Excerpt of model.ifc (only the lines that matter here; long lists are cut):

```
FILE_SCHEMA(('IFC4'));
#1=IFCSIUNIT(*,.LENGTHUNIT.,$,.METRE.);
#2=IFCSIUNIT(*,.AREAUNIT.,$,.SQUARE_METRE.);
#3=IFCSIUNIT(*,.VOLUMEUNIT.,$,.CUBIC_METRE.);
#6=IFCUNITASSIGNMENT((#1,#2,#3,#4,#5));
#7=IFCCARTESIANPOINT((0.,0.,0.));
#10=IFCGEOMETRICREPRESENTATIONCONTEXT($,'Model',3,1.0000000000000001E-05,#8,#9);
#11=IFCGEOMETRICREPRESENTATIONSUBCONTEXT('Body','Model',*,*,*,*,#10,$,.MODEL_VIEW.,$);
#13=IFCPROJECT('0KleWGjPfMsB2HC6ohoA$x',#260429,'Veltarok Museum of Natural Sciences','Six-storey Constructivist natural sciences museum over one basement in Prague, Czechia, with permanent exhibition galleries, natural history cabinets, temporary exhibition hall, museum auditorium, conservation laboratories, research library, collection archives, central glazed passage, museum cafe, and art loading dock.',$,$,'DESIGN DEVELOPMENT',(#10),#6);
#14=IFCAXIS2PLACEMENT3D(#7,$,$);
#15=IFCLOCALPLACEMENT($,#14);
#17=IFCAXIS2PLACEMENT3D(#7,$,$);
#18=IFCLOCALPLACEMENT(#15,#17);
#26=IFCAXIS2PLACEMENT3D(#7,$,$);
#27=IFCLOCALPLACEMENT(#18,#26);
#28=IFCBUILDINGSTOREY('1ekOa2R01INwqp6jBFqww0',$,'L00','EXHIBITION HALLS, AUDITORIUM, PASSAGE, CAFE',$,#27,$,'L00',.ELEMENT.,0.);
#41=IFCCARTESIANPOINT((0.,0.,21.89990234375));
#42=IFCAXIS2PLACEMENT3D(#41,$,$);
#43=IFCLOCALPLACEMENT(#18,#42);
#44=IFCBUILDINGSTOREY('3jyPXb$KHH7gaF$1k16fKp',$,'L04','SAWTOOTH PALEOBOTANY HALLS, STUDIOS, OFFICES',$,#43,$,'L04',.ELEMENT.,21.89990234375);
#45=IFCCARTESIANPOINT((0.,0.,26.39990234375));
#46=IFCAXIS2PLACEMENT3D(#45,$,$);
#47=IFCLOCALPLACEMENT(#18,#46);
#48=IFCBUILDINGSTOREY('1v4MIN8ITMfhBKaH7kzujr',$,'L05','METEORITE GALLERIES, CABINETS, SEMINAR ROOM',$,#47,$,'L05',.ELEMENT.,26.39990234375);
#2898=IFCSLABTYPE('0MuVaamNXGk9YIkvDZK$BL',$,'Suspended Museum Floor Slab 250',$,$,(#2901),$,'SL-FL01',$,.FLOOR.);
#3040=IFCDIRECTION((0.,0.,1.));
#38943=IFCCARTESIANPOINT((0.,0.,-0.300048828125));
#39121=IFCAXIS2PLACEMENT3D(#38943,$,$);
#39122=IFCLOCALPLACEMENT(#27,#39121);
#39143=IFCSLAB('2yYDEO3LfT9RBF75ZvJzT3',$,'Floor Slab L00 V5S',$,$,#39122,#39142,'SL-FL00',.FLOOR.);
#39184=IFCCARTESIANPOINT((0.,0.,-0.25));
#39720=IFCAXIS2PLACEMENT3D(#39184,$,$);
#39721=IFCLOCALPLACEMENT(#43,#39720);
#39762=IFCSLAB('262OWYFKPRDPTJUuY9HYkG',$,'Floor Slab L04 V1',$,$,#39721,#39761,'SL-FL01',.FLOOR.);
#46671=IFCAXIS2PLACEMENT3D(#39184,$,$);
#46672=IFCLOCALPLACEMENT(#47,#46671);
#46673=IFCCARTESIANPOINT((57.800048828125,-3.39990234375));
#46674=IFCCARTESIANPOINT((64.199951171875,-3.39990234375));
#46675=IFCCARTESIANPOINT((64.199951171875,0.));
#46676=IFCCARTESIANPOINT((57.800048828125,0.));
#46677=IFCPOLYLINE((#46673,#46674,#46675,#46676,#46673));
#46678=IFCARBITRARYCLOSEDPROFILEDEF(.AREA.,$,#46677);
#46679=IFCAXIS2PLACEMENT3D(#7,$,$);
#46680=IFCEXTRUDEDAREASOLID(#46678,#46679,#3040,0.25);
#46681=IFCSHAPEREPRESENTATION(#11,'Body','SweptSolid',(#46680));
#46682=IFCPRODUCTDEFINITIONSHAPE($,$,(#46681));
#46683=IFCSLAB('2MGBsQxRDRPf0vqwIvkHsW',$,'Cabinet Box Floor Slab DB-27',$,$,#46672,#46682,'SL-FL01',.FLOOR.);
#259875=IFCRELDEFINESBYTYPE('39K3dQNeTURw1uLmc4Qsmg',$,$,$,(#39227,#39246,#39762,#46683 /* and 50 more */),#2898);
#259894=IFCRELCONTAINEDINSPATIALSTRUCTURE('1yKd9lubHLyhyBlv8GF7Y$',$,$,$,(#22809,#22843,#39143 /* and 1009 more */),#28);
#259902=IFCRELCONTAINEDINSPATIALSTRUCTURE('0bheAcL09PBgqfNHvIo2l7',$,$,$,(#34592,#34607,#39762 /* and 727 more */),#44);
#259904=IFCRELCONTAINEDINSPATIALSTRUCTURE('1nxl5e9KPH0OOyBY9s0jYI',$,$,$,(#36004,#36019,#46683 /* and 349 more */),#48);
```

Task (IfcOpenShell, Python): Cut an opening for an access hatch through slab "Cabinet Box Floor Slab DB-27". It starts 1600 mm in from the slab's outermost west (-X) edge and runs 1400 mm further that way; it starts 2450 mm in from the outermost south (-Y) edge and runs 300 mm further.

```python
import numpy as np
import ifcopenshell
import ifcopenshell.api.feature
import ifcopenshell.api.geometry
import ifcopenshell.api.root
import ifcopenshell.geom
import ifcopenshell.util.placement
import ifcopenshell.util.representation
import ifcopenshell.util.shape
import ifcopenshell.util.unit

model = ifcopenshell.open("model.ifc")
unit_scale = ifcopenshell.util.unit.calculate_unit_scale(model)
settings = ifcopenshell.geom.settings()


def volume(element):
    """Net volume in cubic metres, openings subtracted."""
    shape = ifcopenshell.geom.create_shape(settings, element)
    return ifcopenshell.util.shape.get_volume(shape.geometry)


slab = model.by_guid("2MGBsQxRDRPf0vqwIvkHsW")
before = volume(slab)

# Extent in the slab's own axes, in metres. The edges named are its -X and -Y sides.
slab_shape = ifcopenshell.geom.create_shape(settings, slab)
vertices = ifcopenshell.util.shape.get_vertices(slab_shape.geometry)
x_min, y_min, bottom = vertices.min(axis=0)
top = vertices[:, 2].max()

opening = ifcopenshell.api.root.create_entity(model, ifc_class="IfcOpeningElement", name="Access hatch opening", predefined_type="OPENING")
context = ifcopenshell.util.representation.get_context(model, "Model", "Body", "MODEL_VIEW")
width, depth = 1.4, 0.3
outline = [(0.0, 0.0), (width, 0.0), (width, depth), (0.0, depth), (0.0, 0.0)]
# Overshoot both faces by 50 mm so the cut is clean.
shape = ifcopenshell.api.geometry.add_slab_representation(
    model, context=context, depth=top - bottom + 0.1, polyline=outline
)
ifcopenshell.api.geometry.assign_representation(model, product=opening, representation=shape)

matrix = ifcopenshell.util.placement.get_local_placement(slab.ObjectPlacement)
matrix[:, 3] = matrix @ np.append(np.array([x_min + 1.6, y_min + 2.45, bottom - 0.05]) / unit_scale, 1.0)
ifcopenshell.api.geometry.edit_object_placement(model, product=opening, matrix=matrix, is_si=False)
ifcopenshell.api.feature.add_feature(model, feature=opening, element=slab)

after = volume(slab)

print(f"slab volume {before:.3f} -> {after:.3f} m3")

model.write("model-out.ifc")
```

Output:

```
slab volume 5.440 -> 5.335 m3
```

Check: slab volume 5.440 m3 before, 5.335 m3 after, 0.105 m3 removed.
